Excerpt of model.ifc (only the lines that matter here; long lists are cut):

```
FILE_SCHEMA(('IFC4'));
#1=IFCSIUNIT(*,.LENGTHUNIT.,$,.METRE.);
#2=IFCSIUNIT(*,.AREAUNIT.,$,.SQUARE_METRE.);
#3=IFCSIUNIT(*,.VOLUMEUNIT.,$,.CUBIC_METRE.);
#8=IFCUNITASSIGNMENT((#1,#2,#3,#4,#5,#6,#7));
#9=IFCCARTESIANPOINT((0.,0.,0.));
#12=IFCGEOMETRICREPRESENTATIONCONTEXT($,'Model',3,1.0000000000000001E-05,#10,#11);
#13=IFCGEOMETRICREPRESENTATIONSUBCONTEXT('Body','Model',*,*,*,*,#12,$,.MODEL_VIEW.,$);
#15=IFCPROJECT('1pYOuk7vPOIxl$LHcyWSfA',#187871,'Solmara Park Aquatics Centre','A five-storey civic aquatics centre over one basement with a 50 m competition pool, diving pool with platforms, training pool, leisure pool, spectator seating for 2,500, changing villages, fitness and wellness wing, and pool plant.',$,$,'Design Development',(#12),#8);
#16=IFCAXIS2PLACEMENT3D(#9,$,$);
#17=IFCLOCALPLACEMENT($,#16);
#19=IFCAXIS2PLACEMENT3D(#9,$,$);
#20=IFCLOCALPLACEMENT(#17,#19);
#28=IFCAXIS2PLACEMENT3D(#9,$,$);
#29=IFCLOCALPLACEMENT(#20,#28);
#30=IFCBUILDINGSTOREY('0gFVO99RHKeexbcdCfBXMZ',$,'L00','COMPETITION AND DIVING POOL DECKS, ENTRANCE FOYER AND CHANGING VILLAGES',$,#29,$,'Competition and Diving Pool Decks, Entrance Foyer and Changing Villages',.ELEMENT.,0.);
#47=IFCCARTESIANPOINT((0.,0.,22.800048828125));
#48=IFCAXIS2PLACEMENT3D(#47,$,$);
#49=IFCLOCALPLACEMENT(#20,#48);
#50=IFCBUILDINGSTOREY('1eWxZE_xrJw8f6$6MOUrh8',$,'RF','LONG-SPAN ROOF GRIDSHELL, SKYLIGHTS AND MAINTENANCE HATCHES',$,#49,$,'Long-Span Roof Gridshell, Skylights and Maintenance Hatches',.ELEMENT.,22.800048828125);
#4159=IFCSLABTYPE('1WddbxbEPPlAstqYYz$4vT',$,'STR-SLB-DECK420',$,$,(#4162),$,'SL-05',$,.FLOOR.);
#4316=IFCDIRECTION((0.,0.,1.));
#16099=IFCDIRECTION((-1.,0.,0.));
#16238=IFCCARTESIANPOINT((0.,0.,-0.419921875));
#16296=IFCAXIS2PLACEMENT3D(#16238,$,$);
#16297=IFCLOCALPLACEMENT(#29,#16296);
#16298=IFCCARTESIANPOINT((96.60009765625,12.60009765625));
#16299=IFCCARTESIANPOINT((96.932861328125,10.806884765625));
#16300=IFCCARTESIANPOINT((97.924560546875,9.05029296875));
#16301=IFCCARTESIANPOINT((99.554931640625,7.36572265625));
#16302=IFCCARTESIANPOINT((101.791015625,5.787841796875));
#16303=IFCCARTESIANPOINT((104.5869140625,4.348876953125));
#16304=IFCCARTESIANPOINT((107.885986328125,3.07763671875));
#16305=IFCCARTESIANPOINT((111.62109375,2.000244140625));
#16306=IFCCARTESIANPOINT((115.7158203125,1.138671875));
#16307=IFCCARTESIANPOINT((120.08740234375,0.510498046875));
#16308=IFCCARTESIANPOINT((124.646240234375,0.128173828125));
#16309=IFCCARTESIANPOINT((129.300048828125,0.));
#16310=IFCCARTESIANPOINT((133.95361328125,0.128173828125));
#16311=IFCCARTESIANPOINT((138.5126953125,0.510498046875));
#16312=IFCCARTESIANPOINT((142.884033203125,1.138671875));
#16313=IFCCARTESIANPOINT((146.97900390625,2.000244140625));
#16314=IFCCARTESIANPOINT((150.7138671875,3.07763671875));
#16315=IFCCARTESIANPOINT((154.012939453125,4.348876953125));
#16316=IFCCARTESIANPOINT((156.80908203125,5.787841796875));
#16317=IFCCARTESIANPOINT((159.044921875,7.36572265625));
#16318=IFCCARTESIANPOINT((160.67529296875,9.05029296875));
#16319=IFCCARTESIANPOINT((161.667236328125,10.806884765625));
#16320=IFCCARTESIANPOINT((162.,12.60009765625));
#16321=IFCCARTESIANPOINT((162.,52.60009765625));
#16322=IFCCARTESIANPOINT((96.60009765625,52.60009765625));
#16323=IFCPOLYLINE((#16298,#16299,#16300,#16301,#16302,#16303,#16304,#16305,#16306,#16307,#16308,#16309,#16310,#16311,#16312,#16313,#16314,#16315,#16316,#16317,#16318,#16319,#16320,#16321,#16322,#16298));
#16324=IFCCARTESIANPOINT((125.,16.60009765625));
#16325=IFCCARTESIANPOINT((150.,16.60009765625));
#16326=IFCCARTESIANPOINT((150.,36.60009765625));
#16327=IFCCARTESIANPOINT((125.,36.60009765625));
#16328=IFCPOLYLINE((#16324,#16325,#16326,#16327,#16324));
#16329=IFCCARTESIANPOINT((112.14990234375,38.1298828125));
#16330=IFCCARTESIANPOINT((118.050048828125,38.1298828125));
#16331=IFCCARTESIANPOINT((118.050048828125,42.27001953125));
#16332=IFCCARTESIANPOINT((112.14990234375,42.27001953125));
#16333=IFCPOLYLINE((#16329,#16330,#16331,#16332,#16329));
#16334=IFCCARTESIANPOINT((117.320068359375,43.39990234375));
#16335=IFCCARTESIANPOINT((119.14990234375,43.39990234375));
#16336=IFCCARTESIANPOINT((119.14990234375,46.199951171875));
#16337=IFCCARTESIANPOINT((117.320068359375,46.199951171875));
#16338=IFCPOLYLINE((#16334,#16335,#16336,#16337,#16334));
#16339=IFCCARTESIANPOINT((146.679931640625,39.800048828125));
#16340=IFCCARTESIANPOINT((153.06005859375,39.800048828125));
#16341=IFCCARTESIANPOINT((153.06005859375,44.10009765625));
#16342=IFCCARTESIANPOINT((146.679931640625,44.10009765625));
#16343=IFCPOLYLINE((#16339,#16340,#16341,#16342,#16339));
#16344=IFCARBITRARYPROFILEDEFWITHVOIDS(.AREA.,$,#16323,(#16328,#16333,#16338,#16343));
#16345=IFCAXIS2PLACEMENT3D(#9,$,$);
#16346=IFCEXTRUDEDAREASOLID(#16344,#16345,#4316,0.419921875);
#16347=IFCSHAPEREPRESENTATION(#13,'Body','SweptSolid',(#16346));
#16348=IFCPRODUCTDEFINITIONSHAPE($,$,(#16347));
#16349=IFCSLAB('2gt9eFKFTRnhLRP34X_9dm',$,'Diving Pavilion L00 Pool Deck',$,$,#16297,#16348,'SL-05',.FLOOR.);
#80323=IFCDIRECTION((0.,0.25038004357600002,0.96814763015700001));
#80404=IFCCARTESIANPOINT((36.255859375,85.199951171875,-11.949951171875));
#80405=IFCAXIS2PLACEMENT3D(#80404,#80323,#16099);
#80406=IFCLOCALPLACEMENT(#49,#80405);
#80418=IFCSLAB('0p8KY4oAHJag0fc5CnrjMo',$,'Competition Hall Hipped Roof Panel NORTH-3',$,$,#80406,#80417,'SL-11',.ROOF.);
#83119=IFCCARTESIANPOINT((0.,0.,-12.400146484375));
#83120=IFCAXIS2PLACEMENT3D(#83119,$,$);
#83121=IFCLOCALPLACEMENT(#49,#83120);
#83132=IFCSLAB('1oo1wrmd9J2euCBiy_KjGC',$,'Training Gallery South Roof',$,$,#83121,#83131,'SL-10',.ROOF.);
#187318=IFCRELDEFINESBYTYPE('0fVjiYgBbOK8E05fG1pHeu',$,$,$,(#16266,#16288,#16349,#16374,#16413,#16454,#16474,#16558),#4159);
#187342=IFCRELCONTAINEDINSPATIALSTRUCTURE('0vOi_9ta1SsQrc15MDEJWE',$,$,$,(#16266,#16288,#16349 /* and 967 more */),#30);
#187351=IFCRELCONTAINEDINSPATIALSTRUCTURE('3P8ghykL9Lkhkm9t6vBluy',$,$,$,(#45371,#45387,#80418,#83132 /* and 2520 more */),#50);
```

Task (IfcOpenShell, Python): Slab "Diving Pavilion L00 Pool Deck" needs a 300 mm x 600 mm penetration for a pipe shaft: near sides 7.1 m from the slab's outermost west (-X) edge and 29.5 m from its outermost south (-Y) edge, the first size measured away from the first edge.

```python
import numpy as np
import ifcopenshell
import ifcopenshell.api.feature
import ifcopenshell.api.geometry
import ifcopenshell.api.root
import ifcopenshell.geom
import ifcopenshell.util.placement
import ifcopenshell.util.representation
import ifcopenshell.util.shape
import ifcopenshell.util.unit

model = ifcopenshell.open("model.ifc")
unit_scale = ifcopenshell.util.unit.calculate_unit_scale(model)
settings = ifcopenshell.geom.settings()


def volume(element):
    """Net volume in cubic metres, openings subtracted."""
    shape = ifcopenshell.geom.create_shape(settings, element)
    return ifcopenshell.util.shape.get_volume(shape.geometry)


slab = model.by_id(16349)
before = volume(slab)

# Extent in the slab's own axes, in metres. The edges named are its -X and -Y sides.
slab_shape = ifcopenshell.geom.create_shape(settings, slab)
vertices = ifcopenshell.util.shape.get_vertices(slab_shape.geometry)
x_min, y_min, bottom = vertices.min(axis=0)
top = vertices[:, 2].max()

opening = ifcopenshell.api.root.create_entity(model, ifc_class="IfcOpeningElement", name="Pipe shaft opening", predefined_type="OPENING")
context = ifcopenshell.util.representation.get_context(model, "Model", "Body", "MODEL_VIEW")
width, depth = 0.3, 0.6
outline = [(0.0, 0.0), (width, 0.0), (width, depth), (0.0, depth), (0.0, 0.0)]
# Overshoot both faces by 50 mm so the cut is clean.
shape = ifcopenshell.api.geometry.add_slab_representation(
    model, context=context, depth=top - bottom + 0.1, polyline=outline
)
ifcopenshell.api.geometry.assign_representation(model, product=opening, representation=shape)

matrix = ifcopenshell.util.placement.get_local_placement(slab.ObjectPlacement)
matrix[:, 3] = matrix @ np.append(np.array([x_min + 7.1, y_min + 29.5, bottom - 0.05]) / unit_scale, 1.0)
ifcopenshell.api.geometry.edit_object_placement(model, product=opening, matrix=matrix, is_si=False)
ifcopenshell.api.feature.add_feature(model, feature=opening, element=slab)

after = volume(slab)

print(f"slab volume {before:.3f} -> {after:.3f} m3")

model.write("model_updated.ifc")
```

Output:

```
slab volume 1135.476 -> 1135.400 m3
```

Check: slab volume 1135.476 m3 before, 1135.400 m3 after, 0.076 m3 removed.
